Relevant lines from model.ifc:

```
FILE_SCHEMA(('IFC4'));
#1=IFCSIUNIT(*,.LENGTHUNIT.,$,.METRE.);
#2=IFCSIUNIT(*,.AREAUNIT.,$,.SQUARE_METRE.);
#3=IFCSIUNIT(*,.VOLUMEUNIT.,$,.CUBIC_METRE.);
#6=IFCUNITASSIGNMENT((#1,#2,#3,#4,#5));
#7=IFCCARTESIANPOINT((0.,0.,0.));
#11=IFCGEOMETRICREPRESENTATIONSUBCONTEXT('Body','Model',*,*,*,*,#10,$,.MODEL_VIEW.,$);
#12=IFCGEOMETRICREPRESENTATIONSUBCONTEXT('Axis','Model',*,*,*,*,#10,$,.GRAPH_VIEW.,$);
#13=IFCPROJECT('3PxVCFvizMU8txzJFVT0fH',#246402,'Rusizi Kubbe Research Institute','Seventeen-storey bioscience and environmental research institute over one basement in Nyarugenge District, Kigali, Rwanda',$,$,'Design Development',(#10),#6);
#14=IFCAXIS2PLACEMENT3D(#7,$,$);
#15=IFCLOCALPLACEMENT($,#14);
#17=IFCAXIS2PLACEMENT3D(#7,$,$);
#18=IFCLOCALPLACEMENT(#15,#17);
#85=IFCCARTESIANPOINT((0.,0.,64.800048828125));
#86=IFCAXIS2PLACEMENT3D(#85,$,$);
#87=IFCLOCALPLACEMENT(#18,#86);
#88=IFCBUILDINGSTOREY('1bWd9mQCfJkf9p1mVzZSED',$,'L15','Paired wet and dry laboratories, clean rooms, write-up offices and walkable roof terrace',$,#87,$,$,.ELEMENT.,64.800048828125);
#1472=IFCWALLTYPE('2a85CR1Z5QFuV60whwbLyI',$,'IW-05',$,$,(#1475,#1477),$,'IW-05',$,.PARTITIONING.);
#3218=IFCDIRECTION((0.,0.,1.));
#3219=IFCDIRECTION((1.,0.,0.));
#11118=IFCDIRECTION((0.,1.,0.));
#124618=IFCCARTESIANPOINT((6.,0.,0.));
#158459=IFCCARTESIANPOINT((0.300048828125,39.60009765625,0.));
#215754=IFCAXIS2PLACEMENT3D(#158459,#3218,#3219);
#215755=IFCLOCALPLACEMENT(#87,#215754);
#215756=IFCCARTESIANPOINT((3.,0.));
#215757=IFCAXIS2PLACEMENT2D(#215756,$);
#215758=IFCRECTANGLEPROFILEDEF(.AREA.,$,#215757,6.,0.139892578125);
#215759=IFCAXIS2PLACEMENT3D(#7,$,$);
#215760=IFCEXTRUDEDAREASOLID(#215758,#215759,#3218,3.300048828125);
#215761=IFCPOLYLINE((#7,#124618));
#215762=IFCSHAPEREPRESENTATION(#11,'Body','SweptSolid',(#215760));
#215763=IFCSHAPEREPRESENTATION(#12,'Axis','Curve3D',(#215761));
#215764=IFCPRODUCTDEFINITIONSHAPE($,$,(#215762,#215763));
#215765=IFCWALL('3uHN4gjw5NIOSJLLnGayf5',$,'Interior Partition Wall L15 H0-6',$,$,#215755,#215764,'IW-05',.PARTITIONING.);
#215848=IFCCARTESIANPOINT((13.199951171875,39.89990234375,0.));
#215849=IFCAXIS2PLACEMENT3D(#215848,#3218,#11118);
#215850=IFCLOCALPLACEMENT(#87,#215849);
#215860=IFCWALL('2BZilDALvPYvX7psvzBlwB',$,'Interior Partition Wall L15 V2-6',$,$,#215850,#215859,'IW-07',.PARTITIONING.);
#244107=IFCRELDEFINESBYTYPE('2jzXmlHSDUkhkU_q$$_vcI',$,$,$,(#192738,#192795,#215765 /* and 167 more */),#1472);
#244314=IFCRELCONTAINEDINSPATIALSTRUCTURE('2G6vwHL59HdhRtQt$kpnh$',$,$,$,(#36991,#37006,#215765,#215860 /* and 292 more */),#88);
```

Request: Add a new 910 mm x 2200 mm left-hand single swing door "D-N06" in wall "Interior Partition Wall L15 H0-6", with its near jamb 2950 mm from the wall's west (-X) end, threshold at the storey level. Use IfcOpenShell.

```python
import numpy as np
import ifcopenshell
import ifcopenshell.api.feature
import ifcopenshell.api.geometry
import ifcopenshell.api.root
import ifcopenshell.api.spatial
import ifcopenshell.geom
import ifcopenshell.util.element
import ifcopenshell.util.placement
import ifcopenshell.util.representation
import ifcopenshell.util.shape
import ifcopenshell.util.unit

model = ifcopenshell.open("model.ifc")
unit_scale = ifcopenshell.util.unit.calculate_unit_scale(model)
settings = ifcopenshell.geom.settings()


def volume(element):
    """Net volume in cubic metres, openings subtracted."""
    shape = ifcopenshell.geom.create_shape(settings, element)
    return ifcopenshell.util.shape.get_volume(shape.geometry)


wall = model.by_guid("3uHN4gjw5NIOSJLLnGayf5")
storey = ifcopenshell.util.element.get_container(wall, ifc_class="IfcBuildingStorey")
context = ifcopenshell.util.representation.get_context(model, "Model", "Body", "MODEL_VIEW")
before = volume(wall)

width, height, from_end, sill = 0.91, 2.2, 2.95, 0.0  # metres

# The wall runs along its own X axis, and the end named is its -X end.
wall_shape = ifcopenshell.geom.create_shape(settings, wall)
x, y, z = ifcopenshell.util.shape.get_vertices(wall_shape.geometry).T
start = x.min() + from_end
face, thickness = float(y.min()), float(y.max() - y.min())
wall_matrix = ifcopenshell.util.placement.get_local_placement(wall.ObjectPlacement)
level = ifcopenshell.util.placement.get_local_placement(storey.ObjectPlacement)[2, 3]


def in_wall(x, y):
    """Placement at x, y metres in the wall's axes, at sill height."""
    matrix = wall_matrix.copy()
    matrix[:, 3] = wall_matrix @ np.array([x / unit_scale, y / unit_scale, 0.0, 1.0])
    matrix[2, 3] = level + sill / unit_scale
    return matrix


# Opening: a box that overshoots both wall faces by 50 mm.
opening = ifcopenshell.api.root.create_entity(model, ifc_class="IfcOpeningElement", predefined_type="OPENING")
box = ifcopenshell.api.geometry.add_wall_representation(
    model, context=context, length=width, height=height, thickness=thickness + 0.1
)
ifcopenshell.api.geometry.assign_representation(model, product=opening, representation=box)
ifcopenshell.api.geometry.edit_object_placement(model, product=opening, matrix=in_wall(start, face - 0.05), is_si=False)
ifcopenshell.api.feature.add_feature(model, feature=opening, element=wall)

door = ifcopenshell.api.root.create_entity(model, ifc_class="IfcDoor", name="D-N06", predefined_type="DOOR")
door.OverallWidth, door.OverallHeight = width / unit_scale, height / unit_scale
door.OperationType = "SINGLE_SWING_LEFT"
body = ifcopenshell.api.geometry.add_door_representation(
    model,
    context=context,
    overall_width=door.OverallWidth,
    overall_height=door.OverallHeight,
    operation_type="SINGLE_SWING_LEFT",
    lining_properties={"LiningDepth": thickness / unit_scale, "ThresholdDepth": thickness / unit_scale},
)
ifcopenshell.api.geometry.assign_representation(model, product=door, representation=body)
ifcopenshell.api.spatial.assign_container(model, products=[door], relating_structure=storey)
ifcopenshell.api.feature.add_filling(model, opening=opening, element=door)

# The lining spans the wall, so the door starts at the wall face.
ifcopenshell.api.geometry.edit_object_placement(model, product=door, matrix=in_wall(start, face), is_si=False)

after = volume(wall)

print(f"wall volume {before:.3f} -> {after:.3f} m3")

model.write("model_v2.ifc")
```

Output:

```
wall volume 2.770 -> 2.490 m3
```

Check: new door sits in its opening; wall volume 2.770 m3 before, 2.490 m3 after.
